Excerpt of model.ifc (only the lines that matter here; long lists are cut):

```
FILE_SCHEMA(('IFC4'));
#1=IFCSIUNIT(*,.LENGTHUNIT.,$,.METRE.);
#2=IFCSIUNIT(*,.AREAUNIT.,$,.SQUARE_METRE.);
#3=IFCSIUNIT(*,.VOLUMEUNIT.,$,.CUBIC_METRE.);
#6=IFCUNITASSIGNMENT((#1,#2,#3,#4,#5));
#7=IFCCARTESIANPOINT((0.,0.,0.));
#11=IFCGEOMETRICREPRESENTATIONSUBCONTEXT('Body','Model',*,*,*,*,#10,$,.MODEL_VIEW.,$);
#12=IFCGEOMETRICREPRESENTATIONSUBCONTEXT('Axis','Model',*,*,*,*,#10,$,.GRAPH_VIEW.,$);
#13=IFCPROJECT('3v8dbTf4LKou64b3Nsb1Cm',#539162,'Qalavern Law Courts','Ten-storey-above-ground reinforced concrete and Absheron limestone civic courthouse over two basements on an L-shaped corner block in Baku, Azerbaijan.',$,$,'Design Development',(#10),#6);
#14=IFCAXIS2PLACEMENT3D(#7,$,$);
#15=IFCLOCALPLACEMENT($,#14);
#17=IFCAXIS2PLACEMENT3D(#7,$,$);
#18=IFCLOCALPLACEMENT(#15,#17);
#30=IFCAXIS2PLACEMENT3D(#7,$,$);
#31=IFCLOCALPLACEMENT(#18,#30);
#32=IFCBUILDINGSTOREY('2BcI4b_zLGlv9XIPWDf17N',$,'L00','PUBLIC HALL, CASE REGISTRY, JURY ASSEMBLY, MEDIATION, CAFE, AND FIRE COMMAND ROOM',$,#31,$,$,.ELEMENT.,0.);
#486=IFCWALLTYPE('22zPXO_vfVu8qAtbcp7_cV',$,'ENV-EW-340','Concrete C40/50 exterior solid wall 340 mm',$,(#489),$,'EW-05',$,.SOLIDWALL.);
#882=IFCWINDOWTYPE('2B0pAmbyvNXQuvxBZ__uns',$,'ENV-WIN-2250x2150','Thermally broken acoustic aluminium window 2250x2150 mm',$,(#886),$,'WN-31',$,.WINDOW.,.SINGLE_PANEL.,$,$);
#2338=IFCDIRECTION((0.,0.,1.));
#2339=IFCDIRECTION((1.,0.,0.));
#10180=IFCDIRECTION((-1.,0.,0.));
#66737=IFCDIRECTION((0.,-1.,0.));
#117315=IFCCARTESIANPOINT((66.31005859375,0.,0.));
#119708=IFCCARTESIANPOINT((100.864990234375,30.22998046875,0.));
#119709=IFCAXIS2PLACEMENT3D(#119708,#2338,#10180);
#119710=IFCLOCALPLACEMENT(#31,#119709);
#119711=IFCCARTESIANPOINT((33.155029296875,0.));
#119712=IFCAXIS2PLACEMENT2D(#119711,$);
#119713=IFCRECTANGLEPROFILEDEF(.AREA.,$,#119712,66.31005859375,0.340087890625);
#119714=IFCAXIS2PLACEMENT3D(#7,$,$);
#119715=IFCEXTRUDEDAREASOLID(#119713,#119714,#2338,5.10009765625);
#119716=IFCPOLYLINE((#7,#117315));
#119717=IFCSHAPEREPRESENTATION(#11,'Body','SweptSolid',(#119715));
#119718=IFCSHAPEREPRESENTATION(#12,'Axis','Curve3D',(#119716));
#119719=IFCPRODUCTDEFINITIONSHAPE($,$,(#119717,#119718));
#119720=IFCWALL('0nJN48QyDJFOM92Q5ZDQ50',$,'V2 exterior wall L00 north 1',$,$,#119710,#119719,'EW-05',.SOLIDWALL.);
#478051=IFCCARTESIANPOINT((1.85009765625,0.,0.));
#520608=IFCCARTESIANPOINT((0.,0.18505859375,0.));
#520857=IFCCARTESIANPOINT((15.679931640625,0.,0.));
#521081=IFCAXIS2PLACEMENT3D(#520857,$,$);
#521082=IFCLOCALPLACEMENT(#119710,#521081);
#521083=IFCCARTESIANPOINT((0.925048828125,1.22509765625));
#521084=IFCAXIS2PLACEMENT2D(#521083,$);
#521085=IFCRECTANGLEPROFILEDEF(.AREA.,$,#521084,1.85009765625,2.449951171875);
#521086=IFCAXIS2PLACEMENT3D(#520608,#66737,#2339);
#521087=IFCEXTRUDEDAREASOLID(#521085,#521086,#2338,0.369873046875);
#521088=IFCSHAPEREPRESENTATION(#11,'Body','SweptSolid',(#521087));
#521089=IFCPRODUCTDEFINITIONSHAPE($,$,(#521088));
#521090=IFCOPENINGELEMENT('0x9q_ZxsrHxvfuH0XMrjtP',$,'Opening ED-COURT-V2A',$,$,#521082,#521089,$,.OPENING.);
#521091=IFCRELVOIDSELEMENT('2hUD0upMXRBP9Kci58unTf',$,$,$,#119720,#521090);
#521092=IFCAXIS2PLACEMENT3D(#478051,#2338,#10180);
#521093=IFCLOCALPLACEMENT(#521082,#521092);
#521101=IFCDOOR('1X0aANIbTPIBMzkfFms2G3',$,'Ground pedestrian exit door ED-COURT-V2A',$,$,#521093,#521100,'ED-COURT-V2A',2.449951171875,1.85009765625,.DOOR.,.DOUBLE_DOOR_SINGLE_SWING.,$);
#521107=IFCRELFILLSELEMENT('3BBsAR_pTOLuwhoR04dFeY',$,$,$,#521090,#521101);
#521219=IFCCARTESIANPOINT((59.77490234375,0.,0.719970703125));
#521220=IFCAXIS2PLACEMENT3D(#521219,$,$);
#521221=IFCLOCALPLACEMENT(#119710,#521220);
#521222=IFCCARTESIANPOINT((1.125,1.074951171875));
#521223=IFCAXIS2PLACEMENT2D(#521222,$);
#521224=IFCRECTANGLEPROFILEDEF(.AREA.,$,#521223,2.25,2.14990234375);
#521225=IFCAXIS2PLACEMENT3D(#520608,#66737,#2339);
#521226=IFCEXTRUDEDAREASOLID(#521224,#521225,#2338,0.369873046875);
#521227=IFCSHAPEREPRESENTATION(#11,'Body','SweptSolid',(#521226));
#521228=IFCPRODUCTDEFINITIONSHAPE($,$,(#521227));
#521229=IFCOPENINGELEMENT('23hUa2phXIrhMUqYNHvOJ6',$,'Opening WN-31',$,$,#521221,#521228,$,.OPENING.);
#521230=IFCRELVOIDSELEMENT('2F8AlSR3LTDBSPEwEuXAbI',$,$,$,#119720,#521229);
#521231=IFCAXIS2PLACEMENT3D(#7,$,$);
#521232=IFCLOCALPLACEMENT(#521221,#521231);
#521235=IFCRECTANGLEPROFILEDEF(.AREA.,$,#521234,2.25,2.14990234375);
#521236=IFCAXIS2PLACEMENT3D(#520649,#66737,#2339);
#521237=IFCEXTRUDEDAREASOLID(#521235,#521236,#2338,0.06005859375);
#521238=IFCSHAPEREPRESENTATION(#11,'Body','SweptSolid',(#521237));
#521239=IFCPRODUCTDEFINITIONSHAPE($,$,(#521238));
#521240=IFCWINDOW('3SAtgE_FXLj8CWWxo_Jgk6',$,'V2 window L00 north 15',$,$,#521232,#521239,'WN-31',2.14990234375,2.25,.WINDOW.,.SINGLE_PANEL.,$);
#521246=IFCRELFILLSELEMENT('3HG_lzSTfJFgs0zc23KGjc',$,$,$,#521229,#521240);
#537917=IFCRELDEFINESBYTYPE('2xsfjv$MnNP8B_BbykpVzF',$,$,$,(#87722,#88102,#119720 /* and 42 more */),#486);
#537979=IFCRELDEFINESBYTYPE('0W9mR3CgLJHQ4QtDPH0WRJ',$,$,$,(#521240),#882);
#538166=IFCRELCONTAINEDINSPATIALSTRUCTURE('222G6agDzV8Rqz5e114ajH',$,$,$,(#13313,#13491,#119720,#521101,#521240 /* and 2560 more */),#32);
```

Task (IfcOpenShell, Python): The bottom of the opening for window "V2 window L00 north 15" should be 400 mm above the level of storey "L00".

```python
import numpy as np
import ifcopenshell
import ifcopenshell.api.geometry
import ifcopenshell.geom
import ifcopenshell.util.element
import ifcopenshell.util.placement
import ifcopenshell.util.shape
import ifcopenshell.util.unit

model = ifcopenshell.open("model.ifc")
unit_scale = ifcopenshell.util.unit.calculate_unit_scale(model)

window = model.by_id(521240)
opening = window.FillsVoids[0].RelatingOpeningElement
storey = ifcopenshell.util.element.get_container(window, ifc_class="IfcBuildingStorey")
level = ifcopenshell.util.placement.get_local_placement(storey.ObjectPlacement)[2, 3]

# The opening's origin need not be at the sill, so measure its lowest point.
shape = ifcopenshell.geom.create_shape(ifcopenshell.geom.settings(), opening)
bottom = ifcopenshell.util.shape.get_shape_bottom_elevation(shape, shape.geometry) / unit_scale
dz = level + 0.4 / unit_scale - bottom

shift = np.array([0.0, 0.0, dz])
# The window is placed relative to its opening, so it follows when the opening moves.
matrix = ifcopenshell.util.placement.get_local_placement(opening.ObjectPlacement)
matrix[:3, 3] += shift
ifcopenshell.api.geometry.edit_object_placement(
    model, product=opening, matrix=matrix, is_si=False, should_transform_children=True
)

print(f"moved by {dz * unit_scale:+.3f} m")

model.write("model-out.ifc")
```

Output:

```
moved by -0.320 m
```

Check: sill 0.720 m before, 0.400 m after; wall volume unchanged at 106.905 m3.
